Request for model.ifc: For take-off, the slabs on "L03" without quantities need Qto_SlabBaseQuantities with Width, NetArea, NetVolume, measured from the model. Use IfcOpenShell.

First a look at what the model holds.

```python
import ifcopenshell
import ifcopenshell.util.element
import ifcopenshell.util.unit

model = ifcopenshell.open("model.ifc")
print(model.schema)
for unit_type in ("LENGTHUNIT", "AREAUNIT", "VOLUMEUNIT"):
    print(unit_type, ifcopenshell.util.unit.calculate_unit_scale(model, unit_type))
storey = next(s for s in model.by_type("IfcBuildingStorey") if s.Name == "L03")
slabs = [e for e in ifcopenshell.util.element.get_decomposition(storey) if e.is_a("IfcSlab")]
for e in sorted(slabs, key=lambda e: e.id()):
    print(e.id(), e.is_a(), e.Name, list(ifcopenshell.util.element.get_psets(e, qtos_only=True)), sep=" | ")
```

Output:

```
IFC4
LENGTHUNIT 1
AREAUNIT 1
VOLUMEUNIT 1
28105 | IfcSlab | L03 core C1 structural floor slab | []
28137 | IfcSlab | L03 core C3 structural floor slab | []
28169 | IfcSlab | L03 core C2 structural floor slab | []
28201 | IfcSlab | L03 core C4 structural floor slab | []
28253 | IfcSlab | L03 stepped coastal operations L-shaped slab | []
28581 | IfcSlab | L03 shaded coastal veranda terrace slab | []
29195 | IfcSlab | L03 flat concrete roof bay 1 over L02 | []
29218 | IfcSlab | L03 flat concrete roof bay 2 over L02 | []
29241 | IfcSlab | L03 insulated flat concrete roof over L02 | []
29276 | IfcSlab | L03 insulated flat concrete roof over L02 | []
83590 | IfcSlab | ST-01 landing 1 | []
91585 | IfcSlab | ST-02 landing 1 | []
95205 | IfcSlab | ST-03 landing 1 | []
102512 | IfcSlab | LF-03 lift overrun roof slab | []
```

```python
import ifcopenshell
import ifcopenshell.api.pset
import ifcopenshell.geom
import ifcopenshell.util.element
import ifcopenshell.util.shape
import ifcopenshell.util.unit

model = ifcopenshell.open("model.ifc")
unit_scale = ifcopenshell.util.unit.calculate_unit_scale(model)
area_scale = ifcopenshell.util.unit.calculate_unit_scale(model, "AREAUNIT")
volume_scale = ifcopenshell.util.unit.calculate_unit_scale(model, "VOLUMEUNIT")
settings = ifcopenshell.geom.settings()

storey = next(s for s in model.by_type("IfcBuildingStorey") if s.Name == "L03")
slabs = [e for e in ifcopenshell.util.element.get_decomposition(storey) if e.is_a("IfcSlab")]

for e in sorted(slabs, key=lambda e: e.id()):
    if ifcopenshell.util.element.get_psets(e, qtos_only=True, should_inherit=False):
        continue
    # Geometry comes back in metres, in the element's own axes.
    shape = ifcopenshell.geom.create_shape(settings, e)
    values = {
        "Width": ifcopenshell.util.shape.get_z(shape.geometry) / unit_scale,
        "NetArea": ifcopenshell.util.shape.get_footprint_area(shape.geometry) / area_scale,
        "NetVolume": ifcopenshell.util.shape.get_volume(shape.geometry) / volume_scale,
    }
    qto = ifcopenshell.api.pset.add_qto(model, product=e, name="Qto_SlabBaseQuantities")
    ifcopenshell.api.pset.edit_qto(model, qto=qto, properties=values)
    print(e.id(), {k: round(v, 3) for k, v in values.items()})

model.write("model_edited.ifc")
```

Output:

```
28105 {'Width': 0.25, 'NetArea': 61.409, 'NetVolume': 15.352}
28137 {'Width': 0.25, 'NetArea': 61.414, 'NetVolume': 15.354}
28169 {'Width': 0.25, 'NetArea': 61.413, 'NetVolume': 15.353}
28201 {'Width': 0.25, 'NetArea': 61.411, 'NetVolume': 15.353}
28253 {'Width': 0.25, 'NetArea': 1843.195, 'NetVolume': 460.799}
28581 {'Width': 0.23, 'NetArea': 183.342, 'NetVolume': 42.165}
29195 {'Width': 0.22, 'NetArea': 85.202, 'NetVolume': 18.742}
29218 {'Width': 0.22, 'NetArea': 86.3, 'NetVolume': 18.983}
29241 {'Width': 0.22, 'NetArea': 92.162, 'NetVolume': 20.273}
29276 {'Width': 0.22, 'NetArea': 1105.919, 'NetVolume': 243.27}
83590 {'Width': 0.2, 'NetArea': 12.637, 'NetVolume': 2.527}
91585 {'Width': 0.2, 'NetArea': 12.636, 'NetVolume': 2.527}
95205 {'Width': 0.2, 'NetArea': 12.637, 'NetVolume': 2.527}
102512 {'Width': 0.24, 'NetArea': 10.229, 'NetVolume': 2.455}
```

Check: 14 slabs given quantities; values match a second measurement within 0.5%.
